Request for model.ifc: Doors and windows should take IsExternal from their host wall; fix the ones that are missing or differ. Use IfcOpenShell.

First a look at what the model holds.

```python
import ifcopenshell
import ifcopenshell.util.element

model = ifcopenshell.open("model.ifc")
print(model.schema)
seen = {}
for e in model.by_type("IfcDoor") + model.by_type("IfcWindow"):
    if not e.FillsVoids:
        continue
    host = e.FillsVoids[0].RelatingOpeningElement.VoidsElements[0].RelatingBuildingElement
    own = ifcopenshell.util.element.get_pset(e, f"Pset_{e.is_a()[3:].removesuffix('StandardCase')}Common", "IsExternal")
    wall = ifcopenshell.util.element.get_pset(host, "Pset_WallCommon", "IsExternal")
    seen[e.is_a(), own, wall] = seen.get((e.is_a(), own, wall), 0) + 1
for (cls, own, wall), count in sorted(seen.items(), key=str):
    print(count, cls, "IsExternal:", own, "| host wall:", wall)
```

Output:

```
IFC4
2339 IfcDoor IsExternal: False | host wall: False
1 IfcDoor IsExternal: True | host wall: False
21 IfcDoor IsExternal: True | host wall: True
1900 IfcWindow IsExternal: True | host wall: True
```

```python
import ifcopenshell
import ifcopenshell.api.pset
import ifcopenshell.util.element

model = ifcopenshell.open("model.ifc")

count = 0
for ifc_class, pset_name in (("IfcDoor", "Pset_DoorCommon"), ("IfcWindow", "Pset_WindowCommon")):
    for e in model.by_type(ifc_class):
        if not e.FillsVoids:
            continue
        host = e.FillsVoids[0].RelatingOpeningElement.VoidsElements[0].RelatingBuildingElement
        external = ifcopenshell.util.element.get_pset(host, "Pset_WallCommon", "IsExternal")
        if external is None or ifcopenshell.util.element.get_pset(e, pset_name, "IsExternal") == external:
            continue
        found = ifcopenshell.util.element.get_pset(e, pset_name, should_inherit=False)
        if found:
            pset = model.by_id(found["id"])
            if len(ifcopenshell.util.element.get_elements_by_pset(pset)) > 1:
                pset = ifcopenshell.api.pset.unshare_pset(model, products=[e], pset=pset)[0]
        else:
            pset = ifcopenshell.api.pset.add_pset(model, product=e, name=pset_name)
        ifcopenshell.api.pset.edit_pset(model, pset=pset, properties={"IsExternal": external})
        count += 1

print(count, "updated")

model.write("model_edited.ifc")
```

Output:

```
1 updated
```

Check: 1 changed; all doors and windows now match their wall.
